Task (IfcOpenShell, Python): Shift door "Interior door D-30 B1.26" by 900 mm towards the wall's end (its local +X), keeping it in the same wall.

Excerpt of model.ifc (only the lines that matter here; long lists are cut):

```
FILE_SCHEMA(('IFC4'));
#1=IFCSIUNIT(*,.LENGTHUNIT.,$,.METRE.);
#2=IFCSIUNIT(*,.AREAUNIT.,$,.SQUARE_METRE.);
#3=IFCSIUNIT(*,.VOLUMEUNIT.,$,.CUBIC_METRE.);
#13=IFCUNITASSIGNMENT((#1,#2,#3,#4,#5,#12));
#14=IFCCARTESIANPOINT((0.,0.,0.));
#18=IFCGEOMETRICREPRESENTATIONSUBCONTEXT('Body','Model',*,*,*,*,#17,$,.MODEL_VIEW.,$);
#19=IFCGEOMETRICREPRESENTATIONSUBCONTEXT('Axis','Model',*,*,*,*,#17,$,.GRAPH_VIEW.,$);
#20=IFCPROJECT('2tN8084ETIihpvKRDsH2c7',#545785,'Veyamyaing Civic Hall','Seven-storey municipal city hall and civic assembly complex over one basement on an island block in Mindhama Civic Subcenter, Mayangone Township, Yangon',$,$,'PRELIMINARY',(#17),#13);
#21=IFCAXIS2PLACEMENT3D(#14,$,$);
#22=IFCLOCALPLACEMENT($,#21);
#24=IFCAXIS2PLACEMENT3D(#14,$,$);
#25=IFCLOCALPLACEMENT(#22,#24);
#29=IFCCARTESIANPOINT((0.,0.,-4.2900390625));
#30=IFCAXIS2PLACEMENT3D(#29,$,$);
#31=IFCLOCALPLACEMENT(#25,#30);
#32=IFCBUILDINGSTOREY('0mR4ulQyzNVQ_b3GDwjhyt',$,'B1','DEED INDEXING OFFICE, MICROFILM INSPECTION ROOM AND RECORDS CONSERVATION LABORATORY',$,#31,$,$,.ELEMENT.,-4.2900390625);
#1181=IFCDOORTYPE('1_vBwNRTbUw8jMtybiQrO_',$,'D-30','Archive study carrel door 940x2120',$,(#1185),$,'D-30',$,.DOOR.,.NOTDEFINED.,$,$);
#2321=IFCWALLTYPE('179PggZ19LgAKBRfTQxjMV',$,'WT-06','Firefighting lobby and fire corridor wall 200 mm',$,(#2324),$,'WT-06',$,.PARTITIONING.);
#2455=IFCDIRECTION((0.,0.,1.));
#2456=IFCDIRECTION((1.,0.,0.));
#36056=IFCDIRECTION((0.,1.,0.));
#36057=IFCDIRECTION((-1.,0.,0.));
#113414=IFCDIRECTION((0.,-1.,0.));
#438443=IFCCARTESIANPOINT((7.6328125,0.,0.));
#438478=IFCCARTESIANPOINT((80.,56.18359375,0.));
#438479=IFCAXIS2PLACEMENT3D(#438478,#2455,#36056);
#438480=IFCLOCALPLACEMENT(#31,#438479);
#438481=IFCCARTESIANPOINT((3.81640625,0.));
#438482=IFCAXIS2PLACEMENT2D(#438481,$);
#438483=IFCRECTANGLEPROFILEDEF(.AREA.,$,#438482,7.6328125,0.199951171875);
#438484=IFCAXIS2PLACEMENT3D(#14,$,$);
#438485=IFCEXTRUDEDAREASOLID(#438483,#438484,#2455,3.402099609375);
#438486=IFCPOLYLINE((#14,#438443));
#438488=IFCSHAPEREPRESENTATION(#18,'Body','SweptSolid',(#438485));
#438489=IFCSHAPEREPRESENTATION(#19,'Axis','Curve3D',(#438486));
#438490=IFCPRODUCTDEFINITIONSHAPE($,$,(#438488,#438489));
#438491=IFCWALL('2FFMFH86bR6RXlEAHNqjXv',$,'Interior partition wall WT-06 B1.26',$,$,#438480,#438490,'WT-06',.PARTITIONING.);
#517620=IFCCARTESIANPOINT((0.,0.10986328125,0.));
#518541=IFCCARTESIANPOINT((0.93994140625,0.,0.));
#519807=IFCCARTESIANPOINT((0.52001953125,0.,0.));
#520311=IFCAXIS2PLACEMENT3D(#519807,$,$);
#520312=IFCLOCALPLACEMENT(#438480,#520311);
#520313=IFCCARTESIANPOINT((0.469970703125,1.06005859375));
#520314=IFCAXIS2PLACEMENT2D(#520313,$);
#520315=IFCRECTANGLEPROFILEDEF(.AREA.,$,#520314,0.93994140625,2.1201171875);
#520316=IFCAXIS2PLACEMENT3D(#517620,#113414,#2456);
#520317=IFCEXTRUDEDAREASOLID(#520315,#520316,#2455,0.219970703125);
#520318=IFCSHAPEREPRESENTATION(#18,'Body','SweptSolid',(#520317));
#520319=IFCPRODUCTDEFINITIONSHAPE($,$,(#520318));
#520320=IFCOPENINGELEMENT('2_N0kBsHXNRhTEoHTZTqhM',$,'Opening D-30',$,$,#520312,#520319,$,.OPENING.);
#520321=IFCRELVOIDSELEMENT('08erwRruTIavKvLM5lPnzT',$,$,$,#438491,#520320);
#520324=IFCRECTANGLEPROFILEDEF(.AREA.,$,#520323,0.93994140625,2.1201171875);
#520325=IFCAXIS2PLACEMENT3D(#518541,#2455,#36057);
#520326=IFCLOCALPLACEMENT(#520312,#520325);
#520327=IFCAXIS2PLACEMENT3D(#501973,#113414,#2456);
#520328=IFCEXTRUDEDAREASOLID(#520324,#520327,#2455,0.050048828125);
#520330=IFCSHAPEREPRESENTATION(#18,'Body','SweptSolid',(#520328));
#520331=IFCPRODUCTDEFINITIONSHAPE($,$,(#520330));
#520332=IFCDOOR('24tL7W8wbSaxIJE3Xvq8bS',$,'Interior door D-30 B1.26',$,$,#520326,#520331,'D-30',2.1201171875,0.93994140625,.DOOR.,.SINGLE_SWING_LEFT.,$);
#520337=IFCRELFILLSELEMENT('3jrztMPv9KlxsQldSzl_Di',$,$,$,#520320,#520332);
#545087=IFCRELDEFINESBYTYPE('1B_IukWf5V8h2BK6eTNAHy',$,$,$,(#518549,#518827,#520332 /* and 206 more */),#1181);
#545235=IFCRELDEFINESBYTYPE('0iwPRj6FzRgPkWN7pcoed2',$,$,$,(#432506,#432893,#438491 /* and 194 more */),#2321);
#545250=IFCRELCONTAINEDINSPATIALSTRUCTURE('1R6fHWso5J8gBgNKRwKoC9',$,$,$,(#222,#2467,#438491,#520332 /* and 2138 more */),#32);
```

```python
import ifcopenshell
import ifcopenshell.api.geometry
import ifcopenshell.util.placement
import ifcopenshell.util.unit

model = ifcopenshell.open("model.ifc")
unit_scale = ifcopenshell.util.unit.calculate_unit_scale(model)

door = model.by_id(520332)
opening = door.FillsVoids[0].RelatingOpeningElement
wall = opening.VoidsElements[0].RelatingBuildingElement

wall_matrix = ifcopenshell.util.placement.get_local_placement(wall.ObjectPlacement)
shift = wall_matrix[:3, 0] * 0.9 / unit_scale
before = ifcopenshell.util.placement.get_local_placement(door.ObjectPlacement)[:3, 3].copy()

# The door is placed relative to its opening, so it follows when the opening moves.
matrix = ifcopenshell.util.placement.get_local_placement(opening.ObjectPlacement)
matrix[:3, 3] += shift
ifcopenshell.api.geometry.edit_object_placement(
    model, product=opening, matrix=matrix, is_si=False, should_transform_children=True
)

after = ifcopenshell.util.placement.get_local_placement(door.ObjectPlacement)[:3, 3]
print("door moved by", (after - before).round(3) + 0.0)

model.write("model_v2.ifc")
```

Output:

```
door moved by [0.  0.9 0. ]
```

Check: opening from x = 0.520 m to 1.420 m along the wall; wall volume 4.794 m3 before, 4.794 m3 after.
